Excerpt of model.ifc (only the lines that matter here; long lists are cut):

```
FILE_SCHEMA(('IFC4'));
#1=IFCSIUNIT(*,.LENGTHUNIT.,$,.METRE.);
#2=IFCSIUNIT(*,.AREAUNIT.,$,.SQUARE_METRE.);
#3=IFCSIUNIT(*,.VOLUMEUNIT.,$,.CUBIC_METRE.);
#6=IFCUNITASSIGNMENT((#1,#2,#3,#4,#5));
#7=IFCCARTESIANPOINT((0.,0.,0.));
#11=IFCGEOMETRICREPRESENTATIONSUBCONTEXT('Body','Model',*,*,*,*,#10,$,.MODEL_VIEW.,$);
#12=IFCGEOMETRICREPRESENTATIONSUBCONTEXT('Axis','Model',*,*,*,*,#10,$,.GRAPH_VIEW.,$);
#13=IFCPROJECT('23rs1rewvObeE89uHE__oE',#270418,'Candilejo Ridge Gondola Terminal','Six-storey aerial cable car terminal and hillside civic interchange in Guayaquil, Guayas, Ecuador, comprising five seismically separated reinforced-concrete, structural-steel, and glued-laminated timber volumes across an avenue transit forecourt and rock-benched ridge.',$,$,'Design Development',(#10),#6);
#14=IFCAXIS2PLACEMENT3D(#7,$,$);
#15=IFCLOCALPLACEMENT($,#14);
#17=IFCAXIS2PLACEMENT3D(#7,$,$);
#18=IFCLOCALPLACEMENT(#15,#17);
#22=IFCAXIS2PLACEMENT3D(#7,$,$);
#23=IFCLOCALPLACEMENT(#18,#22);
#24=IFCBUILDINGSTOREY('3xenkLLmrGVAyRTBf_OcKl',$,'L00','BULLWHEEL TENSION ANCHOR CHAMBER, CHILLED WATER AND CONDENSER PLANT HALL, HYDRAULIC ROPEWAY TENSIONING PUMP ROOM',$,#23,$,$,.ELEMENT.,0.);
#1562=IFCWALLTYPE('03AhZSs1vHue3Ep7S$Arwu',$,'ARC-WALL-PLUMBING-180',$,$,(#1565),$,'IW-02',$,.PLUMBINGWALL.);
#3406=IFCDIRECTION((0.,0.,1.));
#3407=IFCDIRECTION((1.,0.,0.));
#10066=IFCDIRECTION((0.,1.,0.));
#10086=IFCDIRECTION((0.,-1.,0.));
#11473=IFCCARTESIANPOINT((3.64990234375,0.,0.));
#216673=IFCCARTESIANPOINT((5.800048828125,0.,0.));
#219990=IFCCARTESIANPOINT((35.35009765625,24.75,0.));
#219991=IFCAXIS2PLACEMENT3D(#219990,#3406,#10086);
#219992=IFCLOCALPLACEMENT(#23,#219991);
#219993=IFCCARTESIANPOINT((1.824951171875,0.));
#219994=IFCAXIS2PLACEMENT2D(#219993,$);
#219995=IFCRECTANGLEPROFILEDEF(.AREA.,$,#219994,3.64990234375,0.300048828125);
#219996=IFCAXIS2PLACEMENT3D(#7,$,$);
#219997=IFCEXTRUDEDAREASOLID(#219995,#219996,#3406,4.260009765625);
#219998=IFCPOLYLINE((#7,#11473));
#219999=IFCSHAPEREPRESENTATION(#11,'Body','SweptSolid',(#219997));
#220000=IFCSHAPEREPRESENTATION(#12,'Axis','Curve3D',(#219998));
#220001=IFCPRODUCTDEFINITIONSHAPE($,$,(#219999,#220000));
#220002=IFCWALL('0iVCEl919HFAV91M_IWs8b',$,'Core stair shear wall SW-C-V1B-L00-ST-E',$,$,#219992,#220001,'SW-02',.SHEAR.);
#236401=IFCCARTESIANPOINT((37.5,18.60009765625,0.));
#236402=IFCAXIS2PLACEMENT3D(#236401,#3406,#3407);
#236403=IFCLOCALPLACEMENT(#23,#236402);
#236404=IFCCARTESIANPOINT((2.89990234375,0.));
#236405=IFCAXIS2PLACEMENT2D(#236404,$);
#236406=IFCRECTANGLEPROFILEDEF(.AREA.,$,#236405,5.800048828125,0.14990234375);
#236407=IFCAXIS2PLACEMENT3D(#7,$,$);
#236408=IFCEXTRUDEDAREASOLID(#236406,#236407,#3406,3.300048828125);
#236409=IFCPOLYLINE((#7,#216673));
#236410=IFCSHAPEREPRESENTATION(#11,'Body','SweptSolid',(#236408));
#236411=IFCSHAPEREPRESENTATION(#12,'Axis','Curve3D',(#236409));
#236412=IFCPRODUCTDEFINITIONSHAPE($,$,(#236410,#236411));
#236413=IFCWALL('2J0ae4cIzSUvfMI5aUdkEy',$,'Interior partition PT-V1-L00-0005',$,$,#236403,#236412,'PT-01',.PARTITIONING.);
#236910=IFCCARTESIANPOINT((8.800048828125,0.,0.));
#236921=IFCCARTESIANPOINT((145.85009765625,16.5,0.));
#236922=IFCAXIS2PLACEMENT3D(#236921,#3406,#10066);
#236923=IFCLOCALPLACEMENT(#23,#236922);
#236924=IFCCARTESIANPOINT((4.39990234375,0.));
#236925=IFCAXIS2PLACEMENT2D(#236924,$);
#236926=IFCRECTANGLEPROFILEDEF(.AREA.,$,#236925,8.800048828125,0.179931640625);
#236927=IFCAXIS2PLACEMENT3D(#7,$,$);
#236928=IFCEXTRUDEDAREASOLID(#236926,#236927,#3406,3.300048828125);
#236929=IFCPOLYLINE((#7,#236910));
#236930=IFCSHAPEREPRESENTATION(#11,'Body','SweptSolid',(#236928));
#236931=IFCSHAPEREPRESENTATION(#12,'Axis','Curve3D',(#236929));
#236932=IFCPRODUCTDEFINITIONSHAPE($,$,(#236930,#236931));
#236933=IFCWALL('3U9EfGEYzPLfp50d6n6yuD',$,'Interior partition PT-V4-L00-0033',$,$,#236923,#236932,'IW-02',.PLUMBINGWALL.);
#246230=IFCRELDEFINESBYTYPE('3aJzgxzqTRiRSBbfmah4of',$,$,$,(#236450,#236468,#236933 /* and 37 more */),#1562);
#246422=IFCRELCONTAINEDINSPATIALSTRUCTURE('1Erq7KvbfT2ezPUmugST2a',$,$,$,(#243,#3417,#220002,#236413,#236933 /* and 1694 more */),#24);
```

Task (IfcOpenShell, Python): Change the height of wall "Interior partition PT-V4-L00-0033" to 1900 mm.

```python
import ifcopenshell
import ifcopenshell.geom
import ifcopenshell.util.representation
import ifcopenshell.util.shape

model = ifcopenshell.open("model.ifc")
settings = ifcopenshell.geom.settings()


def volume(element):
    """Net volume in cubic metres, openings subtracted."""
    shape = ifcopenshell.geom.create_shape(settings, element)
    return ifcopenshell.util.shape.get_volume(shape.geometry)


wall = model.by_guid("3U9EfGEYzPLfp50d6n6yuD")
before = volume(wall)

body = ifcopenshell.util.representation.get_representation(wall, "Model", "Body")
solid = body.Items[0]
old_height = solid.Depth
solid.Depth = 1.9
after = volume(wall)

print(f"height {old_height:g} -> {solid.Depth:g}, volume {before:.3f} -> {after:.3f} m3")

model.write("model_updated.ifc")
```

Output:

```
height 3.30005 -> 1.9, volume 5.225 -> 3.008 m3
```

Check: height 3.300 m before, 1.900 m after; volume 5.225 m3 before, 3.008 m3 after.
